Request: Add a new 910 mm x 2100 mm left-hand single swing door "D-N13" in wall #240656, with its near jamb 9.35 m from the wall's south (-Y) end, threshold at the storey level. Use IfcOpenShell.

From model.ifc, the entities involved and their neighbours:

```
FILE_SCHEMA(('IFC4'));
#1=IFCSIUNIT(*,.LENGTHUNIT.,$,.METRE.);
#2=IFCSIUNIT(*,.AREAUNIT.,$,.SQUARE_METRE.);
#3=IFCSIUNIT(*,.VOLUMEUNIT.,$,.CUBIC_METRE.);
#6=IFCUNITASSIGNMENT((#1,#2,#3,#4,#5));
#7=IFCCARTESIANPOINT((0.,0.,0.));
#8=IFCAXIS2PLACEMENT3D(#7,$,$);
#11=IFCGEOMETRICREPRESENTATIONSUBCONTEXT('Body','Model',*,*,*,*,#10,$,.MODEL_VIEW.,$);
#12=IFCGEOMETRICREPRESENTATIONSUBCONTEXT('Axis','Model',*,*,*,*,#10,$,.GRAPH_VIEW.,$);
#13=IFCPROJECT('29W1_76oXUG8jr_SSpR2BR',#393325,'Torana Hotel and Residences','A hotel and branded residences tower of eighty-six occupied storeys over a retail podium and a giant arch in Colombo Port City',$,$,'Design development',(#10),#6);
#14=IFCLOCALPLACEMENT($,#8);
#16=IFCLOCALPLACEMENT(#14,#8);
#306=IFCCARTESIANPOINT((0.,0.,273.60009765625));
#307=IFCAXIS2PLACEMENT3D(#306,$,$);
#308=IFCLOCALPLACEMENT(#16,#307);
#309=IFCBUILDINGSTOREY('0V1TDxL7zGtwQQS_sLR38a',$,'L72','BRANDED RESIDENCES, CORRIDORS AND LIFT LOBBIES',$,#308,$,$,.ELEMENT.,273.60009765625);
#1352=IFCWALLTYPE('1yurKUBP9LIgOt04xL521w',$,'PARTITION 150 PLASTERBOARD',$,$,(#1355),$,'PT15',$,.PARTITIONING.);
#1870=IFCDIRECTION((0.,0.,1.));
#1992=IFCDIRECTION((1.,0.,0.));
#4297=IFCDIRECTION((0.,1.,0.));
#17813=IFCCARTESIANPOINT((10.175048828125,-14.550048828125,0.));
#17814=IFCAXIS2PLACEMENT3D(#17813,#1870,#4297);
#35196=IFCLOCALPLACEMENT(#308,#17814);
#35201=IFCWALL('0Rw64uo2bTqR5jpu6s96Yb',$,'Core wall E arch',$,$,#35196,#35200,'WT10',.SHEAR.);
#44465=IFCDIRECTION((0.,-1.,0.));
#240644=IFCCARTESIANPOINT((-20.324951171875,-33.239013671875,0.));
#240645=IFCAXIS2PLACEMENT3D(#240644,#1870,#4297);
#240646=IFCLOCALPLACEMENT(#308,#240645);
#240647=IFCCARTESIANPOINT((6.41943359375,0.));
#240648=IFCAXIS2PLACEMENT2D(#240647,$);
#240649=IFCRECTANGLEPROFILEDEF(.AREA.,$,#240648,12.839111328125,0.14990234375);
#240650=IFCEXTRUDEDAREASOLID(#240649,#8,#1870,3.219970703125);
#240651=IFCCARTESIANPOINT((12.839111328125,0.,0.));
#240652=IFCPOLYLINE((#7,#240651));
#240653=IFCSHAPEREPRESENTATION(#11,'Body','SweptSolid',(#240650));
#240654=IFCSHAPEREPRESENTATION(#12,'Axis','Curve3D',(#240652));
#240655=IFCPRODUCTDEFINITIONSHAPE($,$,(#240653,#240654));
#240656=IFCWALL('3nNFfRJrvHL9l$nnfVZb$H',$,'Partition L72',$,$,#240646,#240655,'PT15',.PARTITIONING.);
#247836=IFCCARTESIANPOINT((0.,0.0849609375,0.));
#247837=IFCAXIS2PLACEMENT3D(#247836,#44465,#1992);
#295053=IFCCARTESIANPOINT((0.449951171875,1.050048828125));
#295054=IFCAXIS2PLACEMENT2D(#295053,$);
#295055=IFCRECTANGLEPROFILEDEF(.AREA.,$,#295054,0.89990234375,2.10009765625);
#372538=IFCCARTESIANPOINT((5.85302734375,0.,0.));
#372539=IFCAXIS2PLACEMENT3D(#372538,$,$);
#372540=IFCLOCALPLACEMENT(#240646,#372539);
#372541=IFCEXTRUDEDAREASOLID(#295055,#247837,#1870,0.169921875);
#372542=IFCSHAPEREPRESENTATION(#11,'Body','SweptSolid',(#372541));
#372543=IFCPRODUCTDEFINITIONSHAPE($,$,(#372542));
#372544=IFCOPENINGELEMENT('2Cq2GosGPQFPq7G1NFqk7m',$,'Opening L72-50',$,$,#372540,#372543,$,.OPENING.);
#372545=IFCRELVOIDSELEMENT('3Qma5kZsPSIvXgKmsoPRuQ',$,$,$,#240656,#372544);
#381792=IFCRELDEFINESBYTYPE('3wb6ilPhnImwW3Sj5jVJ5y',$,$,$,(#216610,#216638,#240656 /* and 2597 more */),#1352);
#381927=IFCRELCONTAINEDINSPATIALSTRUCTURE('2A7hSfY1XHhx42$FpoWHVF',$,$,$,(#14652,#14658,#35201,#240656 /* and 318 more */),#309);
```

```python
import numpy as np
import ifcopenshell
import ifcopenshell.api.feature
import ifcopenshell.api.geometry
import ifcopenshell.api.root
import ifcopenshell.api.spatial
import ifcopenshell.geom
import ifcopenshell.util.element
import ifcopenshell.util.placement
import ifcopenshell.util.representation
import ifcopenshell.util.shape
import ifcopenshell.util.unit

model = ifcopenshell.open("model.ifc")
unit_scale = ifcopenshell.util.unit.calculate_unit_scale(model)
settings = ifcopenshell.geom.settings()


def volume(element):
    """Net volume in cubic metres, openings subtracted."""
    shape = ifcopenshell.geom.create_shape(settings, element)
    return ifcopenshell.util.shape.get_volume(shape.geometry)


wall = model.by_guid("3nNFfRJrvHL9l$nnfVZb$H")
storey = ifcopenshell.util.element.get_container(wall, ifc_class="IfcBuildingStorey")
context = ifcopenshell.util.representation.get_context(model, "Model", "Body", "MODEL_VIEW")
before = volume(wall)

width, height, from_end, sill = 0.91, 2.1, 9.35, 0.0  # metres

# The wall runs along its own X axis, and the end named is its -X end.
wall_shape = ifcopenshell.geom.create_shape(settings, wall)
x, y, z = ifcopenshell.util.shape.get_vertices(wall_shape.geometry).T
start = x.min() + from_end
face, thickness = float(y.min()), float(y.max() - y.min())
wall_matrix = ifcopenshell.util.placement.get_local_placement(wall.ObjectPlacement)
level = ifcopenshell.util.placement.get_local_placement(storey.ObjectPlacement)[2, 3]


def in_wall(x, y):
    """Placement at x, y metres in the wall's axes, at sill height."""
    matrix = wall_matrix.copy()
    matrix[:, 3] = wall_matrix @ np.array([x / unit_scale, y / unit_scale, 0.0, 1.0])
    matrix[2, 3] = level + sill / unit_scale
    return matrix


# Opening: a box that overshoots both wall faces by 50 mm.
opening = ifcopenshell.api.root.create_entity(model, ifc_class="IfcOpeningElement", predefined_type="OPENING")
box = ifcopenshell.api.geometry.add_wall_representation(
    model, context=context, length=width, height=height, thickness=thickness + 0.1
)
ifcopenshell.api.geometry.assign_representation(model, product=opening, representation=box)
ifcopenshell.api.geometry.edit_object_placement(model, product=opening, matrix=in_wall(start, face - 0.05), is_si=False)
ifcopenshell.api.feature.add_feature(model, feature=opening, element=wall)

door = ifcopenshell.api.root.create_entity(model, ifc_class="IfcDoor", name="D-N13", predefined_type="DOOR")
door.OverallWidth, door.OverallHeight = width / unit_scale, height / unit_scale
door.OperationType = "SINGLE_SWING_LEFT"
body = ifcopenshell.api.geometry.add_door_representation(
    model,
    context=context,
    overall_width=door.OverallWidth,
    overall_height=door.OverallHeight,
    operation_type="SINGLE_SWING_LEFT",
    lining_properties={"LiningDepth": thickness / unit_scale, "ThresholdDepth": thickness / unit_scale},
)
ifcopenshell.api.geometry.assign_representation(model, product=door, representation=body)
ifcopenshell.api.spatial.assign_container(model, products=[door], relating_structure=storey)
ifcopenshell.api.feature.add_filling(model, opening=opening, element=door)

# The lining spans the wall, so the door starts at the wall face.
ifcopenshell.api.geometry.edit_object_placement(model, product=door, matrix=in_wall(start, face), is_si=False)

after = volume(wall)

print(f"wall volume {before:.3f} -> {after:.3f} m3")

model.write("model_edited.ifc")
```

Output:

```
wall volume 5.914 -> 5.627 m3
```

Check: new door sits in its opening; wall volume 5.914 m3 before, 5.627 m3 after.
